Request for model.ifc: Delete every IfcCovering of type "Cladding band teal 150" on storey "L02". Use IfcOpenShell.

First a look at what the model holds.

```python
import ifcopenshell
import ifcopenshell.util.element

model = ifcopenshell.open("model.ifc")
print(model.schema)
storey = next(s for s in model.by_type("IfcBuildingStorey") if s.Name == "L02")
coverings = [e for e in ifcopenshell.util.element.get_decomposition(storey) if e.is_a("IfcCovering")]
seen = {}
for e in coverings:
    element_type = ifcopenshell.util.element.get_type(e)
    name = element_type.Name if element_type not in (None, e) else None
    seen[name] = seen.get(name, 0) + 1
for name, count in sorted(seen.items(), key=str):
    print(count, "x", name)
```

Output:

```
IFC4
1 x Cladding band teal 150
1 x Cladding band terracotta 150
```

```python
import ifcopenshell
import ifcopenshell.api.root
import ifcopenshell.util.element

model = ifcopenshell.open("model.ifc")

storey = next(s for s in model.by_type("IfcBuildingStorey") if s.Name == "L02")
coverings = [e for e in ifcopenshell.util.element.get_decomposition(storey) if e.is_a("IfcCovering")]
targets = [e for e in coverings if (t := ifcopenshell.util.element.get_type(e)) not in (None, e) and t.Name == "Cladding band teal 150"]

for e in targets:
    ifcopenshell.api.root.remove_product(model, product=e)
print(len(targets), "removed")

model.write("model_rev.ifc")
```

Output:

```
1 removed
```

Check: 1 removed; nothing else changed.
